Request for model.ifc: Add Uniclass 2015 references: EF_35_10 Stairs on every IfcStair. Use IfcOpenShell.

First a look at what the model holds.

```python
import ifcopenshell

model = ifcopenshell.open("model.ifc")
print(model.schema)
print("classifications:", [c.Name for c in model.by_type("IfcClassification")])
for ifc_class in ("IfcDoor", "IfcRoof", "IfcStair", "IfcWall", "IfcWindow"):
    print(ifc_class, len(model.by_type(ifc_class)))
```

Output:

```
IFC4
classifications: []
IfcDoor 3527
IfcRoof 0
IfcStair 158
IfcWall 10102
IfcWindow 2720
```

```python
import ifcopenshell
import ifcopenshell.api.classification

model = ifcopenshell.open("model.ifc")

system = ifcopenshell.api.classification.add_classification(model, classification="Uniclass 2015")

codes = {
    "IfcStair": ("EF_35_10", "Stairs"),
}
for ifc_class, (code, name) in codes.items():
    products = model.by_type(ifc_class)
    ifcopenshell.api.classification.add_reference(
        model, products=products, classification=system, identification=code, name=name
    )
    print(code, len(products))

model.write("model-out.ifc")
```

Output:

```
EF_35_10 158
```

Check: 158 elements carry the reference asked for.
